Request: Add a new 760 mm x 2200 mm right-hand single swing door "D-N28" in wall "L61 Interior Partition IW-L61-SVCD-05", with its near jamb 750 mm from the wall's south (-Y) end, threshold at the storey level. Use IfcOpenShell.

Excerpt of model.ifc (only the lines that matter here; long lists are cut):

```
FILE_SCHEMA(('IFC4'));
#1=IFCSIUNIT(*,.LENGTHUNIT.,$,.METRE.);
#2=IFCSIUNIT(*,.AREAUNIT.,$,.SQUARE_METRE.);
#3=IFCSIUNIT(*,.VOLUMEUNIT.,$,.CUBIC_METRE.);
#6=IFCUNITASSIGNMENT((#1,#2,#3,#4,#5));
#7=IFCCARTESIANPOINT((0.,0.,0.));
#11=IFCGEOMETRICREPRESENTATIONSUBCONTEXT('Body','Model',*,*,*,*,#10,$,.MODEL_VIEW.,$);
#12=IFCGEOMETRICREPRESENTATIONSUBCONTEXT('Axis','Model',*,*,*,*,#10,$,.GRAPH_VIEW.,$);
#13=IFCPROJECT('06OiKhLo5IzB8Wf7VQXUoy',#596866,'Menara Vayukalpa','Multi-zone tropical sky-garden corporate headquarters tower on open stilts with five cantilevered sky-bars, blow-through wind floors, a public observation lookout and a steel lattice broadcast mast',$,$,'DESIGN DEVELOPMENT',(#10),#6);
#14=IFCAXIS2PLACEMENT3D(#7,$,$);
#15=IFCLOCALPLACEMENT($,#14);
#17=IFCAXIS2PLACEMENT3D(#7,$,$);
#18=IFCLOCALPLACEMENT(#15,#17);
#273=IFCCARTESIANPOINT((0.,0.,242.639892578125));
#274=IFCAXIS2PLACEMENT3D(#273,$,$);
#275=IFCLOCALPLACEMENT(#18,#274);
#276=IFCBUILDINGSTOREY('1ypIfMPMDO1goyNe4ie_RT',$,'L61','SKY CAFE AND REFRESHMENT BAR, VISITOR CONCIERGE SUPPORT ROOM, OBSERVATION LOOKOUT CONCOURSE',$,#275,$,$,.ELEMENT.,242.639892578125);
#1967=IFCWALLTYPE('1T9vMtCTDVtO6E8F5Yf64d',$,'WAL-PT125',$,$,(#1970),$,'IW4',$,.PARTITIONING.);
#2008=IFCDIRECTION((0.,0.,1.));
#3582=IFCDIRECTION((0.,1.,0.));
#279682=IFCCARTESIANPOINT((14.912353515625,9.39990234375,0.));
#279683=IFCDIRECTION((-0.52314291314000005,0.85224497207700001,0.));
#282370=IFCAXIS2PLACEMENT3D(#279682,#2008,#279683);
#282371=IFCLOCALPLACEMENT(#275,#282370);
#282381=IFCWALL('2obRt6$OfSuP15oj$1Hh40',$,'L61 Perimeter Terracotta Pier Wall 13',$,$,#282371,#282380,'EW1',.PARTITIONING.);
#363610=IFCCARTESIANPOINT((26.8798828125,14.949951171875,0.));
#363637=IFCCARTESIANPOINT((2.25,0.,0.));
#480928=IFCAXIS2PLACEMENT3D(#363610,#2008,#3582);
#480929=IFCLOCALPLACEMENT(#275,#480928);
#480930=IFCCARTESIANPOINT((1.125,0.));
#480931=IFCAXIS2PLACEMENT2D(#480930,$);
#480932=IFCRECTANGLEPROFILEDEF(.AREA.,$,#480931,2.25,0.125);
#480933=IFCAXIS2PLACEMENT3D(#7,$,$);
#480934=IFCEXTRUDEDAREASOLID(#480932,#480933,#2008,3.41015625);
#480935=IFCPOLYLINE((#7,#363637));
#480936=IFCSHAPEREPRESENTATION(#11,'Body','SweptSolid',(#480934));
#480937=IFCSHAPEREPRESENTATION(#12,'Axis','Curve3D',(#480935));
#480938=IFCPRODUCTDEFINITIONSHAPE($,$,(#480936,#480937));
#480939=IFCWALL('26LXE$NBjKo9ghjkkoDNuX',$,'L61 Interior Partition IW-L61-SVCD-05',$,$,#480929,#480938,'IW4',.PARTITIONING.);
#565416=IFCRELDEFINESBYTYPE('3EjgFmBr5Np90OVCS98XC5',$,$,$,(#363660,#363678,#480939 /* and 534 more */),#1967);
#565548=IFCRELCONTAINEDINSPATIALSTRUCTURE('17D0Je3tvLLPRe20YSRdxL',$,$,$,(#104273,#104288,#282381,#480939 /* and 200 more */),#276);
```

```python
import numpy as np
import ifcopenshell
import ifcopenshell.api.feature
import ifcopenshell.api.geometry
import ifcopenshell.api.root
import ifcopenshell.api.spatial
import ifcopenshell.geom
import ifcopenshell.util.element
import ifcopenshell.util.placement
import ifcopenshell.util.representation
import ifcopenshell.util.shape
import ifcopenshell.util.unit

model = ifcopenshell.open("model.ifc")
unit_scale = ifcopenshell.util.unit.calculate_unit_scale(model)
settings = ifcopenshell.geom.settings()


def volume(element):
    """Net volume in cubic metres, openings subtracted."""
    shape = ifcopenshell.geom.create_shape(settings, element)
    return ifcopenshell.util.shape.get_volume(shape.geometry)


wall = model.by_guid("26LXE$NBjKo9ghjkkoDNuX")
storey = ifcopenshell.util.element.get_container(wall, ifc_class="IfcBuildingStorey")
context = ifcopenshell.util.representation.get_context(model, "Model", "Body", "MODEL_VIEW")
before = volume(wall)

width, height, from_end, sill = 0.76, 2.2, 0.75, 0.0  # metres

# The wall runs along its own X axis, and the end named is its -X end.
wall_shape = ifcopenshell.geom.create_shape(settings, wall)
x, y, z = ifcopenshell.util.shape.get_vertices(wall_shape.geometry).T
start = x.min() + from_end
face, thickness = float(y.min()), float(y.max() - y.min())
wall_matrix = ifcopenshell.util.placement.get_local_placement(wall.ObjectPlacement)
level = ifcopenshell.util.placement.get_local_placement(storey.ObjectPlacement)[2, 3]


def in_wall(x, y):
    """Placement at x, y metres in the wall's axes, at sill height."""
    matrix = wall_matrix.copy()
    matrix[:, 3] = wall_matrix @ np.array([x / unit_scale, y / unit_scale, 0.0, 1.0])
    matrix[2, 3] = level + sill / unit_scale
    return matrix


# Opening: a box that overshoots both wall faces by 50 mm.
opening = ifcopenshell.api.root.create_entity(model, ifc_class="IfcOpeningElement", predefined_type="OPENING")
box = ifcopenshell.api.geometry.add_wall_representation(
    model, context=context, length=width, height=height, thickness=thickness + 0.1
)
ifcopenshell.api.geometry.assign_representation(model, product=opening, representation=box)
ifcopenshell.api.geometry.edit_object_placement(model, product=opening, matrix=in_wall(start, face - 0.05), is_si=False)
ifcopenshell.api.feature.add_feature(model, feature=opening, element=wall)

door = ifcopenshell.api.root.create_entity(model, ifc_class="IfcDoor", name="D-N28", predefined_type="DOOR")
door.OverallWidth, door.OverallHeight = width / unit_scale, height / unit_scale
door.OperationType = "SINGLE_SWING_RIGHT"
body = ifcopenshell.api.geometry.add_door_representation(
    model,
    context=context,
    overall_width=door.OverallWidth,
    overall_height=door.OverallHeight,
    operation_type="SINGLE_SWING_RIGHT",
    lining_properties={"LiningDepth": thickness / unit_scale, "ThresholdDepth": thickness / unit_scale},
)
ifcopenshell.api.geometry.assign_representation(model, product=door, representation=body)
ifcopenshell.api.spatial.assign_container(model, products=[door], relating_structure=storey)
ifcopenshell.api.feature.add_filling(model, opening=opening, element=door)

# The lining spans the wall, so the door starts at the wall face.
ifcopenshell.api.geometry.edit_object_placement(model, product=door, matrix=in_wall(start, face), is_si=False)

after = volume(wall)

print(f"wall volume {before:.3f} -> {after:.3f} m3")

model.write("model_rev.ifc")
```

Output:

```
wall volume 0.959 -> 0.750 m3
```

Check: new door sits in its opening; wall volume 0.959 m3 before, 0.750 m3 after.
